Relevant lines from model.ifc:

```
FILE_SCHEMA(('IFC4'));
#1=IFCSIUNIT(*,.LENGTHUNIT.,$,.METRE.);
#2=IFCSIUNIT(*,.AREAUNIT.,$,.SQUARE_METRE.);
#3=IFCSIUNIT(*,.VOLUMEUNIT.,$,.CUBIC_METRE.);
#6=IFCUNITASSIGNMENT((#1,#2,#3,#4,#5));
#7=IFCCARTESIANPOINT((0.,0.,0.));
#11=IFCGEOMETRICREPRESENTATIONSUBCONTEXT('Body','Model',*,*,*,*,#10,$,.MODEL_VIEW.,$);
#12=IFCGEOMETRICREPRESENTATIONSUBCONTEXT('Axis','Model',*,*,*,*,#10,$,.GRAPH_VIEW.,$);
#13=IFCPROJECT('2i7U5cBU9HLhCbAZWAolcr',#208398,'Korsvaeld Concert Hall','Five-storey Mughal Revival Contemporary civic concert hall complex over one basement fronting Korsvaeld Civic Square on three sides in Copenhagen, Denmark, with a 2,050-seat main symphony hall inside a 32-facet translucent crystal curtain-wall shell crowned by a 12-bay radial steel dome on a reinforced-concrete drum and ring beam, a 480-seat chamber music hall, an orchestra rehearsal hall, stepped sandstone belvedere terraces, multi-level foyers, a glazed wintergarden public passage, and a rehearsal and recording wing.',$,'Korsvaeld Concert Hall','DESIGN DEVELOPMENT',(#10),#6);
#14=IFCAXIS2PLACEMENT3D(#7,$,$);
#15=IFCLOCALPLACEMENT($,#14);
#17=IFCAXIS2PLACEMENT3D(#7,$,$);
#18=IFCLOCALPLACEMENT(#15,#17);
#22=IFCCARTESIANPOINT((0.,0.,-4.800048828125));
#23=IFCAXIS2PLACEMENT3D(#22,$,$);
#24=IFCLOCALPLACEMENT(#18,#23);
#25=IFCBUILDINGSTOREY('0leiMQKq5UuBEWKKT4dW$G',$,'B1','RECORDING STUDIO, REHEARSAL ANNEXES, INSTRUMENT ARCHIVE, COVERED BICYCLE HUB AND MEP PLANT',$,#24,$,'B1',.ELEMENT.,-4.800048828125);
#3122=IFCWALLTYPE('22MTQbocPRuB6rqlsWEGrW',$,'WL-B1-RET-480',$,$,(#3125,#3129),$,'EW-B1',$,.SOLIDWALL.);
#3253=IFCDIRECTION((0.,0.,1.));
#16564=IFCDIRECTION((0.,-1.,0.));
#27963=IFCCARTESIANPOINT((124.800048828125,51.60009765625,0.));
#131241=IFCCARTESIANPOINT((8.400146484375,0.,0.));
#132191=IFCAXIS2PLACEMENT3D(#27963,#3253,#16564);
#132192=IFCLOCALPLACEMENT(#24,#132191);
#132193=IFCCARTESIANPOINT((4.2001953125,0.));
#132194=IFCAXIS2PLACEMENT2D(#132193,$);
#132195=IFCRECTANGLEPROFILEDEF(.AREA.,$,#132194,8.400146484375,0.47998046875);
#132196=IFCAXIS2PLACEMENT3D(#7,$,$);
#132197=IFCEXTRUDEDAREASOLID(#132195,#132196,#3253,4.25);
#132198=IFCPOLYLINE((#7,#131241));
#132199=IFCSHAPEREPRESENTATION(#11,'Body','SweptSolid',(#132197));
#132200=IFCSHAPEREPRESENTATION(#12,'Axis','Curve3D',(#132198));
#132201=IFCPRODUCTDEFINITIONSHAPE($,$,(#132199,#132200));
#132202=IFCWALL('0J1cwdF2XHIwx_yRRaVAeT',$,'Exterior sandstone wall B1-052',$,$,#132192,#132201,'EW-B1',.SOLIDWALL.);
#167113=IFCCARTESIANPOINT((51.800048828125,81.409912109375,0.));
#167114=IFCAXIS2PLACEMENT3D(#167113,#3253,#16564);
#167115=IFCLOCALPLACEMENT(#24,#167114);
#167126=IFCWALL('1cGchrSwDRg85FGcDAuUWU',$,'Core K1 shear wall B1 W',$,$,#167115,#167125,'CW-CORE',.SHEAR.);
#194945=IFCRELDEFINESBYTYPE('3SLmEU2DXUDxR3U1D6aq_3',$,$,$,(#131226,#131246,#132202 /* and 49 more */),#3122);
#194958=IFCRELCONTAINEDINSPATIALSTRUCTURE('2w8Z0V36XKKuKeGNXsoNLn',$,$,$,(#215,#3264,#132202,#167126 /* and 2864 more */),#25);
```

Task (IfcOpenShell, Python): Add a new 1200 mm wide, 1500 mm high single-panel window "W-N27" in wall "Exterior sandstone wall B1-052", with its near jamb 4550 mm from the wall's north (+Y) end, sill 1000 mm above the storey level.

```python
import numpy as np
import ifcopenshell
import ifcopenshell.api.feature
import ifcopenshell.api.geometry
import ifcopenshell.api.root
import ifcopenshell.api.spatial
import ifcopenshell.geom
import ifcopenshell.util.element
import ifcopenshell.util.placement
import ifcopenshell.util.representation
import ifcopenshell.util.shape
import ifcopenshell.util.unit

model = ifcopenshell.open("model.ifc")
unit_scale = ifcopenshell.util.unit.calculate_unit_scale(model)
settings = ifcopenshell.geom.settings()


def volume(element):
    """Net volume in cubic metres, openings subtracted."""
    shape = ifcopenshell.geom.create_shape(settings, element)
    return ifcopenshell.util.shape.get_volume(shape.geometry)


wall = model.by_guid("0J1cwdF2XHIwx_yRRaVAeT")
storey = ifcopenshell.util.element.get_container(wall, ifc_class="IfcBuildingStorey")
context = ifcopenshell.util.representation.get_context(model, "Model", "Body", "MODEL_VIEW")
before = volume(wall)

width, height, from_end, sill = 1.2, 1.5, 4.55, 1  # metres

# The wall runs along its own X axis, and the end named is its -X end.
wall_shape = ifcopenshell.geom.create_shape(settings, wall)
x, y, z = ifcopenshell.util.shape.get_vertices(wall_shape.geometry).T
start = x.min() + from_end
face, thickness = float(y.min()), float(y.max() - y.min())
wall_matrix = ifcopenshell.util.placement.get_local_placement(wall.ObjectPlacement)
level = ifcopenshell.util.placement.get_local_placement(storey.ObjectPlacement)[2, 3]


def in_wall(x, y):
    """Placement at x, y metres in the wall's axes, at sill height."""
    matrix = wall_matrix.copy()
    matrix[:, 3] = wall_matrix @ np.array([x / unit_scale, y / unit_scale, 0.0, 1.0])
    matrix[2, 3] = level + sill / unit_scale
    return matrix


# Opening: a box that overshoots both wall faces by 50 mm.
opening = ifcopenshell.api.root.create_entity(model, ifc_class="IfcOpeningElement", predefined_type="OPENING")
box = ifcopenshell.api.geometry.add_wall_representation(
    model, context=context, length=width, height=height, thickness=thickness + 0.1
)
ifcopenshell.api.geometry.assign_representation(model, product=opening, representation=box)
ifcopenshell.api.geometry.edit_object_placement(model, product=opening, matrix=in_wall(start, face - 0.05), is_si=False)
ifcopenshell.api.feature.add_feature(model, feature=opening, element=wall)

window = ifcopenshell.api.root.create_entity(model, ifc_class="IfcWindow", name="W-N27", predefined_type="WINDOW")
window.OverallWidth, window.OverallHeight = width / unit_scale, height / unit_scale
window.PartitioningType = "SINGLE_PANEL"
body = ifcopenshell.api.geometry.add_window_representation(
    model,
    context=context,
    overall_width=window.OverallWidth,
    overall_height=window.OverallHeight,
    partition_type="SINGLE_PANEL",
)
ifcopenshell.api.geometry.assign_representation(model, product=window, representation=body)
ifcopenshell.api.spatial.assign_container(model, products=[window], relating_structure=storey)
ifcopenshell.api.feature.add_filling(model, opening=opening, element=window)

# Centre the window in the wall's thickness.
ifcopenshell.api.geometry.edit_object_placement(model, product=window, matrix=in_wall(start, face), is_si=False)
window_shape = ifcopenshell.geom.create_shape(settings, window)
depth = ifcopenshell.util.shape.get_vertices(window_shape.geometry)[:, 1]
offset = face + thickness / 2 - (depth.min() + depth.max()) / 2
ifcopenshell.api.geometry.edit_object_placement(model, product=window, matrix=in_wall(start, offset), is_si=False)

after = volume(wall)

print(f"wall volume {before:.3f} -> {after:.3f} m3")

model.write("model_updated.ifc")
```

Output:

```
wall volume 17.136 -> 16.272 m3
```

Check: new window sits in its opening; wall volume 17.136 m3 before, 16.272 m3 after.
